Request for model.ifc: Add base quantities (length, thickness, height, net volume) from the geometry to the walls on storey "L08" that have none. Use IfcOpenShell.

First a look at what the model holds.

```python
import ifcopenshell
import ifcopenshell.util.element
import ifcopenshell.util.unit

model = ifcopenshell.open("model.ifc")
print(model.schema)
for unit_type in ("LENGTHUNIT", "AREAUNIT", "VOLUMEUNIT"):
    print(unit_type, ifcopenshell.util.unit.calculate_unit_scale(model, unit_type))
storey = next(s for s in model.by_type("IfcBuildingStorey") if s.Name == "L08")
walls = [e for e in ifcopenshell.util.element.get_decomposition(storey) if e.is_a("IfcWall")]
for e in sorted(walls, key=lambda e: e.id()):
    print(e.id(), e.is_a(), e.Name, list(ifcopenshell.util.element.get_psets(e, qtos_only=True)), sep=" | ")
```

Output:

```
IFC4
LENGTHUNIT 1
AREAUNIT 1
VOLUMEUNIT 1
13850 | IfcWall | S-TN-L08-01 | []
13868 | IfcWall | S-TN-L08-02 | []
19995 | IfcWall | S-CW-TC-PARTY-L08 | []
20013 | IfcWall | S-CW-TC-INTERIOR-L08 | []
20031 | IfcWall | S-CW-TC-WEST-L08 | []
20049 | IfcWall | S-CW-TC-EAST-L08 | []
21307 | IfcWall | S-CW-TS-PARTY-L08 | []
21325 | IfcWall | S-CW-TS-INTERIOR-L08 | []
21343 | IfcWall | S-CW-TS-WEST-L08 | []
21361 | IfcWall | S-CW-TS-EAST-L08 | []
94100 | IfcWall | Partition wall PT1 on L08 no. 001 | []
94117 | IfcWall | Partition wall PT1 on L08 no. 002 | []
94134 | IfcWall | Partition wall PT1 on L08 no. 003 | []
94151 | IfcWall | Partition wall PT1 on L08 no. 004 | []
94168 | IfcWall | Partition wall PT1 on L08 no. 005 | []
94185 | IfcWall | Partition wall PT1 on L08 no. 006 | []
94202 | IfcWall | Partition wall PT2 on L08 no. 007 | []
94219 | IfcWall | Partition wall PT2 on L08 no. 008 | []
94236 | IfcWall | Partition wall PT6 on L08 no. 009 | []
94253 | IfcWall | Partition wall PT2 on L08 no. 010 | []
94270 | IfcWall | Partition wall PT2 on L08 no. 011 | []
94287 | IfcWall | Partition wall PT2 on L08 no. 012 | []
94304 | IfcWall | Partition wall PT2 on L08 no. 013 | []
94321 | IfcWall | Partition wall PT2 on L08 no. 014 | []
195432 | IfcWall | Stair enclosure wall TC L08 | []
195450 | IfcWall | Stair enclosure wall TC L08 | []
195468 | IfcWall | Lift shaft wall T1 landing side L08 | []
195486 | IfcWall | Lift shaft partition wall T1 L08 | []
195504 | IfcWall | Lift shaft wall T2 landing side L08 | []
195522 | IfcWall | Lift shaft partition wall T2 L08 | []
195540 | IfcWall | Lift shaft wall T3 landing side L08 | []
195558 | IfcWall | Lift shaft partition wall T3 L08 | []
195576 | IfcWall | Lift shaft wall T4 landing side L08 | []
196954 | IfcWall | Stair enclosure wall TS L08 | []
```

```python
import ifcopenshell
import ifcopenshell.api.pset
import ifcopenshell.geom
import ifcopenshell.util.element
import ifcopenshell.util.shape
import ifcopenshell.util.unit

model = ifcopenshell.open("model.ifc")
unit_scale = ifcopenshell.util.unit.calculate_unit_scale(model)
volume_scale = ifcopenshell.util.unit.calculate_unit_scale(model, "VOLUMEUNIT")
settings = ifcopenshell.geom.settings()

storey = next(s for s in model.by_type("IfcBuildingStorey") if s.Name == "L08")
walls = [e for e in ifcopenshell.util.element.get_decomposition(storey) if e.is_a("IfcWall")]

for e in sorted(walls, key=lambda e: e.id()):
    if ifcopenshell.util.element.get_psets(e, qtos_only=True, should_inherit=False):
        continue
    # Geometry comes back in metres, in the element's own axes.
    shape = ifcopenshell.geom.create_shape(settings, e)
    values = {
        "Length": ifcopenshell.util.shape.get_x(shape.geometry) / unit_scale,
        "Width": ifcopenshell.util.shape.get_y(shape.geometry) / unit_scale,
        "Height": ifcopenshell.util.shape.get_z(shape.geometry) / unit_scale,
        "NetVolume": ifcopenshell.util.shape.get_volume(shape.geometry) / volume_scale,
    }
    qto = ifcopenshell.api.pset.add_qto(model, product=e, name="Qto_WallBaseQuantities")
    ifcopenshell.api.pset.edit_qto(model, qto=qto, properties=values)
    print(e.id(), {k: round(v, 3) for k, v in values.items()})

model.write("model_rev.ifc")
```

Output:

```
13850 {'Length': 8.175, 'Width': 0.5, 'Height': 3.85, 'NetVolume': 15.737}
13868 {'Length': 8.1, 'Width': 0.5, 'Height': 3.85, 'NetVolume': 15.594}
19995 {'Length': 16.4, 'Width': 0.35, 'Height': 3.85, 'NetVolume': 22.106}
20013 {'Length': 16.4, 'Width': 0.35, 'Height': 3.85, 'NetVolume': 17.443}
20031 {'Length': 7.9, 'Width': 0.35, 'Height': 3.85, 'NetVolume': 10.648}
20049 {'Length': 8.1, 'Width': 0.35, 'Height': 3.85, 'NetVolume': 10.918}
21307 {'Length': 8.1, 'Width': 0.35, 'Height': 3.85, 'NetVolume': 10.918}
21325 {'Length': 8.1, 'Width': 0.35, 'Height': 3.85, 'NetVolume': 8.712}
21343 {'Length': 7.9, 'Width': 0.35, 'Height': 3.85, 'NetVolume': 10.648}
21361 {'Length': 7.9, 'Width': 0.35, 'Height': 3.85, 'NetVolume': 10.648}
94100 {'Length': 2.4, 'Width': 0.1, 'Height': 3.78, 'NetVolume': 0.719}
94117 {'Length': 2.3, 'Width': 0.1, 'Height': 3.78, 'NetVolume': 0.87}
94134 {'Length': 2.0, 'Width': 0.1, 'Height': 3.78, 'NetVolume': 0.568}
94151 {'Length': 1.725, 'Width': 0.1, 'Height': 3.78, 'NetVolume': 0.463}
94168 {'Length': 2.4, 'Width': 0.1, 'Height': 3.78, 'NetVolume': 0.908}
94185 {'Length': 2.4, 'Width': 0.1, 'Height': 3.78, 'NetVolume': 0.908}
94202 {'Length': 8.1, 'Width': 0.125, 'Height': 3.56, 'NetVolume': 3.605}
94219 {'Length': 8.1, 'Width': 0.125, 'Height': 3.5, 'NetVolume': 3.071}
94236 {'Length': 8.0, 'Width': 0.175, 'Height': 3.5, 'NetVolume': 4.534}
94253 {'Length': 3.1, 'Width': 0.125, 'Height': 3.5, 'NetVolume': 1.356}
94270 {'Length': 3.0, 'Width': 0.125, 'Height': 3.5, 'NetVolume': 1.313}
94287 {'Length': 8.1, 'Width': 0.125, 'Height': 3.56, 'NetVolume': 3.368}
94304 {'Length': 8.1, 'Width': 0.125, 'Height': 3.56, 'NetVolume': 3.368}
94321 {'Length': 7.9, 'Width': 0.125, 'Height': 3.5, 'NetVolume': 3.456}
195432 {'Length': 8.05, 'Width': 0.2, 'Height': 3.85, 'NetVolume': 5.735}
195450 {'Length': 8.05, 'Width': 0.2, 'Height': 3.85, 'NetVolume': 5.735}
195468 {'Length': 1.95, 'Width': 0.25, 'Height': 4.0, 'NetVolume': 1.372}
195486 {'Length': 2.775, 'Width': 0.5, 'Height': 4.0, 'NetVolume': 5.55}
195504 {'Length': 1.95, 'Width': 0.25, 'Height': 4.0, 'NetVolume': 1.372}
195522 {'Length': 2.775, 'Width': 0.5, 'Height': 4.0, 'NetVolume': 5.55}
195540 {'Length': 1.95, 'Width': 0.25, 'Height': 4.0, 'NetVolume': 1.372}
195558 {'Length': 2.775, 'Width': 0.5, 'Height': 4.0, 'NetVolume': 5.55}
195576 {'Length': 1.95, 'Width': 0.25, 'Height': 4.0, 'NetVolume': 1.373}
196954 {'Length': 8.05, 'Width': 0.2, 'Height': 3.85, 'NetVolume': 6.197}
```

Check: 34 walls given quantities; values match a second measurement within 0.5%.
